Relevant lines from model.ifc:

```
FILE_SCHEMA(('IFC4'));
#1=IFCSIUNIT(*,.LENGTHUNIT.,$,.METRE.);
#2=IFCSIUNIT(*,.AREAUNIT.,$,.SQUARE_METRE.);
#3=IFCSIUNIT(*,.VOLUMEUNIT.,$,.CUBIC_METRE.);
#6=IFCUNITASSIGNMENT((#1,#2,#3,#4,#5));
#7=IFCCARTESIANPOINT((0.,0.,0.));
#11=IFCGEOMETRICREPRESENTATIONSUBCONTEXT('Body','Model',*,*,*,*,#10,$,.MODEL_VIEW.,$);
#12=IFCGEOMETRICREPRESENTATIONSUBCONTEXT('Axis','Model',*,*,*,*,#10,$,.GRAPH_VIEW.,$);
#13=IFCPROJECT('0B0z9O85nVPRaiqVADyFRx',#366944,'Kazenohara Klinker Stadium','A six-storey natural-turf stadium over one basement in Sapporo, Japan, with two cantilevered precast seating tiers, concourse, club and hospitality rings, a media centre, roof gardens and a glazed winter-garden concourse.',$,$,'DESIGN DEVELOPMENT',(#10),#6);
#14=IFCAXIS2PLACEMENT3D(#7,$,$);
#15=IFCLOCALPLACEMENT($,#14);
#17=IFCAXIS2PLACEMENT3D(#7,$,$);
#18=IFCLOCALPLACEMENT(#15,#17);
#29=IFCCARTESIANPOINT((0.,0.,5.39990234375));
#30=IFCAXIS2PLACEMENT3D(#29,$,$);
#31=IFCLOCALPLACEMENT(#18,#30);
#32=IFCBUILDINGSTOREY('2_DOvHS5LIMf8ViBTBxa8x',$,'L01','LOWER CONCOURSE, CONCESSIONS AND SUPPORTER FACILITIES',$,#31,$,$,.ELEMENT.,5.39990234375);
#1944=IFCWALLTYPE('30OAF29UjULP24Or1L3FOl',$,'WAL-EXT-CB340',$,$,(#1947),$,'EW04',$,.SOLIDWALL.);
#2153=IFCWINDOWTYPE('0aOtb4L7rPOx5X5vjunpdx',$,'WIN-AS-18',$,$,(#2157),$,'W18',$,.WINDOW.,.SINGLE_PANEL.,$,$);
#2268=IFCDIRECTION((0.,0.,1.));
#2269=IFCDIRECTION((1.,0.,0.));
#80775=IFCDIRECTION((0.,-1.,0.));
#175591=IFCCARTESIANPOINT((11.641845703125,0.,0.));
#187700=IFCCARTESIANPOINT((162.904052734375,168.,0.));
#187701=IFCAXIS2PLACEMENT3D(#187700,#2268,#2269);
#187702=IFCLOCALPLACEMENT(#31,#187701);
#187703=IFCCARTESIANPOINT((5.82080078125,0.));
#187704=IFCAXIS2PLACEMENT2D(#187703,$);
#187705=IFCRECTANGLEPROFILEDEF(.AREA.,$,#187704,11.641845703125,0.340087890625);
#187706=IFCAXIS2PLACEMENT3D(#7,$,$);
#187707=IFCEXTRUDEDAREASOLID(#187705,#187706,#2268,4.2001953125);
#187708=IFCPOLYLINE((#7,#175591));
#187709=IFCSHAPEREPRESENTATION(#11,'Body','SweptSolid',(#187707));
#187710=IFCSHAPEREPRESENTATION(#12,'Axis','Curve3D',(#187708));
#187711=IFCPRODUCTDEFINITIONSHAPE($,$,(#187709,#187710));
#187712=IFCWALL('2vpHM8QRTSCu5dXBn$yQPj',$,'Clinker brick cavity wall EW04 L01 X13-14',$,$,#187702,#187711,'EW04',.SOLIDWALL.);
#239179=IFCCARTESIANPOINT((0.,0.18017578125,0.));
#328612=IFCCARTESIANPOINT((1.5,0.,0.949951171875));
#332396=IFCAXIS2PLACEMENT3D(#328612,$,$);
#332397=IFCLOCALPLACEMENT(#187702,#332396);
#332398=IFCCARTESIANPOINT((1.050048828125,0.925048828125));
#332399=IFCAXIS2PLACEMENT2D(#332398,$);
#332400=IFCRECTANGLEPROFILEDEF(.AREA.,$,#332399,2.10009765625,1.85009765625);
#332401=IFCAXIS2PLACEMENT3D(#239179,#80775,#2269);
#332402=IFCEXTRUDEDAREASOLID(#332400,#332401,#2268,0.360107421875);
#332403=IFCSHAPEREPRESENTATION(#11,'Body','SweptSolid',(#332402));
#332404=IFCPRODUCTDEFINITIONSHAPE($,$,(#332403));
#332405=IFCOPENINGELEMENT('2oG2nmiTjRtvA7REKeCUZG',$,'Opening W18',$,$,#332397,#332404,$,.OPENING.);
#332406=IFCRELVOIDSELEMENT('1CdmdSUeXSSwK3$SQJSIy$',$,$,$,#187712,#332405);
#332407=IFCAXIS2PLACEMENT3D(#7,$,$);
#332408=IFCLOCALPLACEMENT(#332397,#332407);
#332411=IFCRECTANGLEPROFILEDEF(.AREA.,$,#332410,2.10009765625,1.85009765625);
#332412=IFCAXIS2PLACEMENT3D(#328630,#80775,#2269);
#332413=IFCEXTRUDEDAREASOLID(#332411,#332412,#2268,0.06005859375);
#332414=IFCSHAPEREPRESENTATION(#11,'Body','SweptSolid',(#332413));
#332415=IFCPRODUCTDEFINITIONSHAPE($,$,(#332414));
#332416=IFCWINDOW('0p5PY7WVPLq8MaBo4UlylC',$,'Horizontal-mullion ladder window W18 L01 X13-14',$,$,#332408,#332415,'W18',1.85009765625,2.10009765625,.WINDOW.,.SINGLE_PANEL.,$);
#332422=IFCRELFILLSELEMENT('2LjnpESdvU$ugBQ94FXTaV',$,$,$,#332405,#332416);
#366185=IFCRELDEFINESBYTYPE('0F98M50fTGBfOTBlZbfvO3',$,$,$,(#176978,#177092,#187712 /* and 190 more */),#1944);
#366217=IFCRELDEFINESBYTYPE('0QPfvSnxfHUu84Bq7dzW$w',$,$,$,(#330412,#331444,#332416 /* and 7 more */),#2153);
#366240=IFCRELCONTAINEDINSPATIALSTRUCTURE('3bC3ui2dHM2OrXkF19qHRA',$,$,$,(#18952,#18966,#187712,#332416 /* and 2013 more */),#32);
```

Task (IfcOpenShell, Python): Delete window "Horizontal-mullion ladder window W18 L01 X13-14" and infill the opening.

```python
import ifcopenshell
import ifcopenshell.api.feature
import ifcopenshell.api.root
import ifcopenshell.geom
import ifcopenshell.util.shape

model = ifcopenshell.open("model.ifc")
settings = ifcopenshell.geom.settings()


def volume(element):
    """Net volume in cubic metres, openings subtracted."""
    shape = ifcopenshell.geom.create_shape(settings, element)
    return ifcopenshell.util.shape.get_volume(shape.geometry)


window = model.by_guid("0p5PY7WVPLq8MaBo4UlylC")
opening = window.FillsVoids[0].RelatingOpeningElement
wall = opening.VoidsElements[0].RelatingBuildingElement
before = volume(wall)

ifcopenshell.api.root.remove_product(model, product=window)
ifcopenshell.api.feature.remove_feature(model, feature=opening)

after = volume(wall)

print(f"wall volume {before:.3f} -> {after:.3f} m3")

model.write("model_updated.ifc")
```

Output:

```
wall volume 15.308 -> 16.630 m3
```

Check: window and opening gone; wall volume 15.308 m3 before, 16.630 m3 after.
